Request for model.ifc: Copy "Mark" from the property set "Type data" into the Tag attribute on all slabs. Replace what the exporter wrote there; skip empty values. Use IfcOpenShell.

First a look at what the model holds.

```python
import ifcopenshell
import ifcopenshell.util.element

model = ifcopenshell.open("model.ifc")
print(model.schema)
slabs = model.by_type("IfcSlab")
print(len(slabs), "slabs")
for e in slabs[:8]:
    source = ifcopenshell.util.element.get_pset(e, "Type data", "Mark")
    target = e.Tag
    print(e.id(), repr(source), repr(target), sep=" | ")
```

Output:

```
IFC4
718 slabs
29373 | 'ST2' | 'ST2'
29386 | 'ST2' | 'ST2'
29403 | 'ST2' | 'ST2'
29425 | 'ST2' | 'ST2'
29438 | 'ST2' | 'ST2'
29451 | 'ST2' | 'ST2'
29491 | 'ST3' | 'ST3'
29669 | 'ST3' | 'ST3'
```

```python
import ifcopenshell
import ifcopenshell.util.element

model = ifcopenshell.open("model.ifc")

count = 0
for e in model.by_type("IfcSlab"):
    value = ifcopenshell.util.element.get_pset(e, "Type data", "Mark")
    current = e.Tag
    if not value or not value.strip() or current == value:
        continue
    e.Tag = value
    count += 1

print(count, "slabs updated")

model.write("model_updated.ifc")
```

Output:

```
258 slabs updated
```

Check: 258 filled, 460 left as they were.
